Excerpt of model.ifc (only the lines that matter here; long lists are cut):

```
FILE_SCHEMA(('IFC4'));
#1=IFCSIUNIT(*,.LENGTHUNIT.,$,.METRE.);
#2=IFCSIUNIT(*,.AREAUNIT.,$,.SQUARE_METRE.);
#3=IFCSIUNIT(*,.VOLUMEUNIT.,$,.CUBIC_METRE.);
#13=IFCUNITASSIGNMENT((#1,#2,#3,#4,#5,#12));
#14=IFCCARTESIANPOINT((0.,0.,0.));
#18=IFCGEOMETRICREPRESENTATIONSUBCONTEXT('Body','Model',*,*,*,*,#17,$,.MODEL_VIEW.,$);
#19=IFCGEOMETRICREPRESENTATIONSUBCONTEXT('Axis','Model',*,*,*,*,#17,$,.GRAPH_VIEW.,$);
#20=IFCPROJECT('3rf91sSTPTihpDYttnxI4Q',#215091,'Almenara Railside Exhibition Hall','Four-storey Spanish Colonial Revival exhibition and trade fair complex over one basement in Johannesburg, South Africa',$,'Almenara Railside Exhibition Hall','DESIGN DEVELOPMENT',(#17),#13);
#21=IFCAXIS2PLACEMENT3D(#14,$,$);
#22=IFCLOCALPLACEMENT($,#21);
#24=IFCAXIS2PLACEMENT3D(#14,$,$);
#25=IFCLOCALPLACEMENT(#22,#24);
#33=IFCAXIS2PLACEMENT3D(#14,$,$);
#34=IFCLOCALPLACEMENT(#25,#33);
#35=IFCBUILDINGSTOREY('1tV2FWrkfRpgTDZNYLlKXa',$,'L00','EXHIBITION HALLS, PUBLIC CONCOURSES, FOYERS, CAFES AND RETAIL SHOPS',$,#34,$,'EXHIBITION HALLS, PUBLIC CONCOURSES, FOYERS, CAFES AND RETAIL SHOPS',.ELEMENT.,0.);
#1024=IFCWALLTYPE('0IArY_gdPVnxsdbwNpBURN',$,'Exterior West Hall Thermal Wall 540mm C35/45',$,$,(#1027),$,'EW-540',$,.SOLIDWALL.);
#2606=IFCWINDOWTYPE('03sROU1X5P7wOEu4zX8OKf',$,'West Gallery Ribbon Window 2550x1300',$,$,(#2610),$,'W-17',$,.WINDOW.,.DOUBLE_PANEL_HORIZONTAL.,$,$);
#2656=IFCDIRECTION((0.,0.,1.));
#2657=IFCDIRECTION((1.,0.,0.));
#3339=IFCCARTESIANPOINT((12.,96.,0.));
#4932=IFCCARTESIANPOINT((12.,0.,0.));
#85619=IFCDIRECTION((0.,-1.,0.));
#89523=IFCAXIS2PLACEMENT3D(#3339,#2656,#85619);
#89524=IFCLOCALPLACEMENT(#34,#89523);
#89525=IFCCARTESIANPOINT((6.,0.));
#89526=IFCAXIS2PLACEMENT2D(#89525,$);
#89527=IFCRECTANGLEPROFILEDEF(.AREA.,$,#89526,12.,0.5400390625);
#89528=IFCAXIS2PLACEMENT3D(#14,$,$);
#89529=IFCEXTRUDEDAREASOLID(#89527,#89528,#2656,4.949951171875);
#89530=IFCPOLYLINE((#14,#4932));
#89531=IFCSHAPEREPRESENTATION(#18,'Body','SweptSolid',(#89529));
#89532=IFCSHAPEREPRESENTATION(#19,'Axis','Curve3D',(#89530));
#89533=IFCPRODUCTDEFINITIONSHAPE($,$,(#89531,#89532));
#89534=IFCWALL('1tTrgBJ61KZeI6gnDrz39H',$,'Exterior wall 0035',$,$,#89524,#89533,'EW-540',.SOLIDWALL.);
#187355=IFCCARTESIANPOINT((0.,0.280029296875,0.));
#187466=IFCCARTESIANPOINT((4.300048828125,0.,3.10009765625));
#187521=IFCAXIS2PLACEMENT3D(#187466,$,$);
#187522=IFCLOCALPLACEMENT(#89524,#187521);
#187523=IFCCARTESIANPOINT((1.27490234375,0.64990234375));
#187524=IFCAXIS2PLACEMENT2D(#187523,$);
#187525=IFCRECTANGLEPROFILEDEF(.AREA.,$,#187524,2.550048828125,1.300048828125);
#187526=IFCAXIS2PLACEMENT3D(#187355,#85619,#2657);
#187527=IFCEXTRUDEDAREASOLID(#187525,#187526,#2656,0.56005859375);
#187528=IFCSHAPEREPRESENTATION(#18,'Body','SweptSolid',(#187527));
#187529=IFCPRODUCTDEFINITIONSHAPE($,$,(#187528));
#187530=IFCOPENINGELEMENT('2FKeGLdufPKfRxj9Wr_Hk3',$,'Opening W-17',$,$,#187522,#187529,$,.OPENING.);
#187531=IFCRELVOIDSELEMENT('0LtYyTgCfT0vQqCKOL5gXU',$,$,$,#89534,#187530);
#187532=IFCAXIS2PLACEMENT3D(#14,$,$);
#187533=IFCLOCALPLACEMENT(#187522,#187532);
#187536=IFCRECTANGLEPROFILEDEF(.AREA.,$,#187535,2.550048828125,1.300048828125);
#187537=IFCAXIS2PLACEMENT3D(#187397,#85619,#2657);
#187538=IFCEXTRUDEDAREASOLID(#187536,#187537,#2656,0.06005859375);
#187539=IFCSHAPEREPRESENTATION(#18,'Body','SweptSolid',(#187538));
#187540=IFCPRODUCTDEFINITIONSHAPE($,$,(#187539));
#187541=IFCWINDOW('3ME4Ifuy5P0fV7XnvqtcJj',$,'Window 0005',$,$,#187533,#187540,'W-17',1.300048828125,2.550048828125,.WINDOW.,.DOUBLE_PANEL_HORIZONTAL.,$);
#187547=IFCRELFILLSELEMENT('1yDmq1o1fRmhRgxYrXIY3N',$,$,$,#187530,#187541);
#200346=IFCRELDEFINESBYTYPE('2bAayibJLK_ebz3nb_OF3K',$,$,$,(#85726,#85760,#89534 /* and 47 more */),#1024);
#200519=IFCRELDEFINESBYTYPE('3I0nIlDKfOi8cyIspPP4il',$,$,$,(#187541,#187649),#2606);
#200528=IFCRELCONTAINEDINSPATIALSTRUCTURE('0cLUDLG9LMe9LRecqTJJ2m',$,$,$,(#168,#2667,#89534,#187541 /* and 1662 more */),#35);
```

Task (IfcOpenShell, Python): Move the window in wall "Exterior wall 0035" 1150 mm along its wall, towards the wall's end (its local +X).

```python
import ifcopenshell
import ifcopenshell.api.geometry
import ifcopenshell.util.placement
import ifcopenshell.util.unit

model = ifcopenshell.open("model.ifc")
unit_scale = ifcopenshell.util.unit.calculate_unit_scale(model)

window = model.by_guid("3ME4Ifuy5P0fV7XnvqtcJj")
opening = window.FillsVoids[0].RelatingOpeningElement
wall = opening.VoidsElements[0].RelatingBuildingElement

wall_matrix = ifcopenshell.util.placement.get_local_placement(wall.ObjectPlacement)
shift = wall_matrix[:3, 0] * 1.15 / unit_scale
before = ifcopenshell.util.placement.get_local_placement(window.ObjectPlacement)[:3, 3].copy()

# The window is placed relative to its opening, so it follows when the opening moves.
matrix = ifcopenshell.util.placement.get_local_placement(opening.ObjectPlacement)
matrix[:3, 3] += shift
ifcopenshell.api.geometry.edit_object_placement(
    model, product=opening, matrix=matrix, is_si=False, should_transform_children=True
)

after = ifcopenshell.util.placement.get_local_placement(window.ObjectPlacement)[:3, 3]
print("window moved by", (after - before).round(3) + 0.0)

model.write("model_v2.ifc")
```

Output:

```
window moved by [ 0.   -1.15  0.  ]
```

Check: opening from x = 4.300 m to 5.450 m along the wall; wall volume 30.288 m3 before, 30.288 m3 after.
